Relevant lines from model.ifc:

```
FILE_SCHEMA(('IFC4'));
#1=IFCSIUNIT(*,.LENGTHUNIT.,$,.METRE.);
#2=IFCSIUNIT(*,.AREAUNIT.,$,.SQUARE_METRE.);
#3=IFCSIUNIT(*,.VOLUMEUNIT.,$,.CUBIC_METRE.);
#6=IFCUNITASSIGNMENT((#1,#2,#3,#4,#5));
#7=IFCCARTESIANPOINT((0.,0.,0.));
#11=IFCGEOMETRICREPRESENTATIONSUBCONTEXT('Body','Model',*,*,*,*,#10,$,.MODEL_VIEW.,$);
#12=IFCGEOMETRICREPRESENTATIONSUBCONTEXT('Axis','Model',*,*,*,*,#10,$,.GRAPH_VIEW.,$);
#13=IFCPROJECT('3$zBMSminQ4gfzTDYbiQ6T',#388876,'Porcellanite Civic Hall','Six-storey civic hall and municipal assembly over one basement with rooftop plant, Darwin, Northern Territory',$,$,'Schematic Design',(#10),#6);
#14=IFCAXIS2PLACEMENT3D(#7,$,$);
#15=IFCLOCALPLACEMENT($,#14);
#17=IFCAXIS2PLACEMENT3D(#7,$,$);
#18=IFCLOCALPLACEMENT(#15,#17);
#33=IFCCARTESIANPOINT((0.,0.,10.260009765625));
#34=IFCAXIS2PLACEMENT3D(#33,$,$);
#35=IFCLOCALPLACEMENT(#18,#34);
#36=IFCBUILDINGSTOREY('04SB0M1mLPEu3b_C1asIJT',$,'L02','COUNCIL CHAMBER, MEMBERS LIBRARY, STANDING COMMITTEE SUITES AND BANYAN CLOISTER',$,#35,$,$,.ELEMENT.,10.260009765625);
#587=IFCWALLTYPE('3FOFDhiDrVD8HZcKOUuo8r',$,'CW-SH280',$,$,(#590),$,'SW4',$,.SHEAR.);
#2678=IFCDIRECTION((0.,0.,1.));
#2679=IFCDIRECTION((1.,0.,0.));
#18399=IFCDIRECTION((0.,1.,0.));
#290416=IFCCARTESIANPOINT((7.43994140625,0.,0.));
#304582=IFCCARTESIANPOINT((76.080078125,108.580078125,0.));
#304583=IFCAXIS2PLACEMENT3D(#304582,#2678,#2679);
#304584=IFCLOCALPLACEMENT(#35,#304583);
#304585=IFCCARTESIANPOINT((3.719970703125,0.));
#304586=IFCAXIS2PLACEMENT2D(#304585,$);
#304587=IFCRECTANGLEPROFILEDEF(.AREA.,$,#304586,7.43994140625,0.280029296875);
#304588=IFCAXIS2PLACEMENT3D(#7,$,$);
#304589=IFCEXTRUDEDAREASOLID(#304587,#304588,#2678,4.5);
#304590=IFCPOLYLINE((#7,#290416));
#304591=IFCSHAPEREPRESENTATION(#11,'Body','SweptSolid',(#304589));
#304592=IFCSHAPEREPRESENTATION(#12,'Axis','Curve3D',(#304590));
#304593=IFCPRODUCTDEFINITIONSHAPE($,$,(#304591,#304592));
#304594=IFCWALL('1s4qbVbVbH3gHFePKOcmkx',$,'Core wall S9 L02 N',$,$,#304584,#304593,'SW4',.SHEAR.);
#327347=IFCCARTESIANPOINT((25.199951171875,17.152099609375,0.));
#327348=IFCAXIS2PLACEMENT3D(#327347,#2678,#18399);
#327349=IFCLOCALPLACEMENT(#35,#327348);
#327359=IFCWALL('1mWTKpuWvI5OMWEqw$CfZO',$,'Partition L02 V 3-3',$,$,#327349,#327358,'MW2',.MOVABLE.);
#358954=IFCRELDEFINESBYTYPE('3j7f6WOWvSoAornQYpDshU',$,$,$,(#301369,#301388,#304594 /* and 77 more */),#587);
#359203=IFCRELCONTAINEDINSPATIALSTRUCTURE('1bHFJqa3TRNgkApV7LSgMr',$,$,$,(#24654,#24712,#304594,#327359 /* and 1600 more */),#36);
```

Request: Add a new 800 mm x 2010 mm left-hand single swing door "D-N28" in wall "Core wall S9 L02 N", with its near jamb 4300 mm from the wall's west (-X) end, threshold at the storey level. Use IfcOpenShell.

```python
import numpy as np
import ifcopenshell
import ifcopenshell.api.feature
import ifcopenshell.api.geometry
import ifcopenshell.api.root
import ifcopenshell.api.spatial
import ifcopenshell.geom
import ifcopenshell.util.element
import ifcopenshell.util.placement
import ifcopenshell.util.representation
import ifcopenshell.util.shape
import ifcopenshell.util.unit

model = ifcopenshell.open("model.ifc")
unit_scale = ifcopenshell.util.unit.calculate_unit_scale(model)
settings = ifcopenshell.geom.settings()


def volume(element):
    """Net volume in cubic metres, openings subtracted."""
    shape = ifcopenshell.geom.create_shape(settings, element)
    return ifcopenshell.util.shape.get_volume(shape.geometry)


wall = model.by_guid("1s4qbVbVbH3gHFePKOcmkx")
storey = ifcopenshell.util.element.get_container(wall, ifc_class="IfcBuildingStorey")
context = ifcopenshell.util.representation.get_context(model, "Model", "Body", "MODEL_VIEW")
before = volume(wall)

width, height, from_end, sill = 0.8, 2.01, 4.3, 0.0  # metres

# The wall runs along its own X axis, and the end named is its -X end.
wall_shape = ifcopenshell.geom.create_shape(settings, wall)
x, y, z = ifcopenshell.util.shape.get_vertices(wall_shape.geometry).T
start = x.min() + from_end
face, thickness = float(y.min()), float(y.max() - y.min())
wall_matrix = ifcopenshell.util.placement.get_local_placement(wall.ObjectPlacement)
level = ifcopenshell.util.placement.get_local_placement(storey.ObjectPlacement)[2, 3]


def in_wall(x, y):
    """Placement at x, y metres in the wall's axes, at sill height."""
    matrix = wall_matrix.copy()
    matrix[:, 3] = wall_matrix @ np.array([x / unit_scale, y / unit_scale, 0.0, 1.0])
    matrix[2, 3] = level + sill / unit_scale
    return matrix


# Opening: a box that overshoots both wall faces by 50 mm.
opening = ifcopenshell.api.root.create_entity(model, ifc_class="IfcOpeningElement", predefined_type="OPENING")
box = ifcopenshell.api.geometry.add_wall_representation(
    model, context=context, length=width, height=height, thickness=thickness + 0.1
)
ifcopenshell.api.geometry.assign_representation(model, product=opening, representation=box)
ifcopenshell.api.geometry.edit_object_placement(model, product=opening, matrix=in_wall(start, face - 0.05), is_si=False)
ifcopenshell.api.feature.add_feature(model, feature=opening, element=wall)

door = ifcopenshell.api.root.create_entity(model, ifc_class="IfcDoor", name="D-N28", predefined_type="DOOR")
door.OverallWidth, door.OverallHeight = width / unit_scale, height / unit_scale
door.OperationType = "SINGLE_SWING_LEFT"
body = ifcopenshell.api.geometry.add_door_representation(
    model,
    context=context,
    overall_width=door.OverallWidth,
    overall_height=door.OverallHeight,
    operation_type="SINGLE_SWING_LEFT",
    lining_properties={"LiningDepth": thickness / unit_scale, "ThresholdDepth": thickness / unit_scale},
)
ifcopenshell.api.geometry.assign_representation(model, product=door, representation=body)
ifcopenshell.api.spatial.assign_container(model, products=[door], relating_structure=storey)
ifcopenshell.api.feature.add_filling(model, opening=opening, element=door)

# The lining spans the wall, so the door starts at the wall face.
ifcopenshell.api.geometry.edit_object_placement(model, product=door, matrix=in_wall(start, face), is_si=False)

after = volume(wall)

print(f"wall volume {before:.3f} -> {after:.3f} m3")

model.write("model_edited.ifc")
```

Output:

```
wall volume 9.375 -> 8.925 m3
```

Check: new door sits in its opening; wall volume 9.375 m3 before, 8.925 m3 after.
